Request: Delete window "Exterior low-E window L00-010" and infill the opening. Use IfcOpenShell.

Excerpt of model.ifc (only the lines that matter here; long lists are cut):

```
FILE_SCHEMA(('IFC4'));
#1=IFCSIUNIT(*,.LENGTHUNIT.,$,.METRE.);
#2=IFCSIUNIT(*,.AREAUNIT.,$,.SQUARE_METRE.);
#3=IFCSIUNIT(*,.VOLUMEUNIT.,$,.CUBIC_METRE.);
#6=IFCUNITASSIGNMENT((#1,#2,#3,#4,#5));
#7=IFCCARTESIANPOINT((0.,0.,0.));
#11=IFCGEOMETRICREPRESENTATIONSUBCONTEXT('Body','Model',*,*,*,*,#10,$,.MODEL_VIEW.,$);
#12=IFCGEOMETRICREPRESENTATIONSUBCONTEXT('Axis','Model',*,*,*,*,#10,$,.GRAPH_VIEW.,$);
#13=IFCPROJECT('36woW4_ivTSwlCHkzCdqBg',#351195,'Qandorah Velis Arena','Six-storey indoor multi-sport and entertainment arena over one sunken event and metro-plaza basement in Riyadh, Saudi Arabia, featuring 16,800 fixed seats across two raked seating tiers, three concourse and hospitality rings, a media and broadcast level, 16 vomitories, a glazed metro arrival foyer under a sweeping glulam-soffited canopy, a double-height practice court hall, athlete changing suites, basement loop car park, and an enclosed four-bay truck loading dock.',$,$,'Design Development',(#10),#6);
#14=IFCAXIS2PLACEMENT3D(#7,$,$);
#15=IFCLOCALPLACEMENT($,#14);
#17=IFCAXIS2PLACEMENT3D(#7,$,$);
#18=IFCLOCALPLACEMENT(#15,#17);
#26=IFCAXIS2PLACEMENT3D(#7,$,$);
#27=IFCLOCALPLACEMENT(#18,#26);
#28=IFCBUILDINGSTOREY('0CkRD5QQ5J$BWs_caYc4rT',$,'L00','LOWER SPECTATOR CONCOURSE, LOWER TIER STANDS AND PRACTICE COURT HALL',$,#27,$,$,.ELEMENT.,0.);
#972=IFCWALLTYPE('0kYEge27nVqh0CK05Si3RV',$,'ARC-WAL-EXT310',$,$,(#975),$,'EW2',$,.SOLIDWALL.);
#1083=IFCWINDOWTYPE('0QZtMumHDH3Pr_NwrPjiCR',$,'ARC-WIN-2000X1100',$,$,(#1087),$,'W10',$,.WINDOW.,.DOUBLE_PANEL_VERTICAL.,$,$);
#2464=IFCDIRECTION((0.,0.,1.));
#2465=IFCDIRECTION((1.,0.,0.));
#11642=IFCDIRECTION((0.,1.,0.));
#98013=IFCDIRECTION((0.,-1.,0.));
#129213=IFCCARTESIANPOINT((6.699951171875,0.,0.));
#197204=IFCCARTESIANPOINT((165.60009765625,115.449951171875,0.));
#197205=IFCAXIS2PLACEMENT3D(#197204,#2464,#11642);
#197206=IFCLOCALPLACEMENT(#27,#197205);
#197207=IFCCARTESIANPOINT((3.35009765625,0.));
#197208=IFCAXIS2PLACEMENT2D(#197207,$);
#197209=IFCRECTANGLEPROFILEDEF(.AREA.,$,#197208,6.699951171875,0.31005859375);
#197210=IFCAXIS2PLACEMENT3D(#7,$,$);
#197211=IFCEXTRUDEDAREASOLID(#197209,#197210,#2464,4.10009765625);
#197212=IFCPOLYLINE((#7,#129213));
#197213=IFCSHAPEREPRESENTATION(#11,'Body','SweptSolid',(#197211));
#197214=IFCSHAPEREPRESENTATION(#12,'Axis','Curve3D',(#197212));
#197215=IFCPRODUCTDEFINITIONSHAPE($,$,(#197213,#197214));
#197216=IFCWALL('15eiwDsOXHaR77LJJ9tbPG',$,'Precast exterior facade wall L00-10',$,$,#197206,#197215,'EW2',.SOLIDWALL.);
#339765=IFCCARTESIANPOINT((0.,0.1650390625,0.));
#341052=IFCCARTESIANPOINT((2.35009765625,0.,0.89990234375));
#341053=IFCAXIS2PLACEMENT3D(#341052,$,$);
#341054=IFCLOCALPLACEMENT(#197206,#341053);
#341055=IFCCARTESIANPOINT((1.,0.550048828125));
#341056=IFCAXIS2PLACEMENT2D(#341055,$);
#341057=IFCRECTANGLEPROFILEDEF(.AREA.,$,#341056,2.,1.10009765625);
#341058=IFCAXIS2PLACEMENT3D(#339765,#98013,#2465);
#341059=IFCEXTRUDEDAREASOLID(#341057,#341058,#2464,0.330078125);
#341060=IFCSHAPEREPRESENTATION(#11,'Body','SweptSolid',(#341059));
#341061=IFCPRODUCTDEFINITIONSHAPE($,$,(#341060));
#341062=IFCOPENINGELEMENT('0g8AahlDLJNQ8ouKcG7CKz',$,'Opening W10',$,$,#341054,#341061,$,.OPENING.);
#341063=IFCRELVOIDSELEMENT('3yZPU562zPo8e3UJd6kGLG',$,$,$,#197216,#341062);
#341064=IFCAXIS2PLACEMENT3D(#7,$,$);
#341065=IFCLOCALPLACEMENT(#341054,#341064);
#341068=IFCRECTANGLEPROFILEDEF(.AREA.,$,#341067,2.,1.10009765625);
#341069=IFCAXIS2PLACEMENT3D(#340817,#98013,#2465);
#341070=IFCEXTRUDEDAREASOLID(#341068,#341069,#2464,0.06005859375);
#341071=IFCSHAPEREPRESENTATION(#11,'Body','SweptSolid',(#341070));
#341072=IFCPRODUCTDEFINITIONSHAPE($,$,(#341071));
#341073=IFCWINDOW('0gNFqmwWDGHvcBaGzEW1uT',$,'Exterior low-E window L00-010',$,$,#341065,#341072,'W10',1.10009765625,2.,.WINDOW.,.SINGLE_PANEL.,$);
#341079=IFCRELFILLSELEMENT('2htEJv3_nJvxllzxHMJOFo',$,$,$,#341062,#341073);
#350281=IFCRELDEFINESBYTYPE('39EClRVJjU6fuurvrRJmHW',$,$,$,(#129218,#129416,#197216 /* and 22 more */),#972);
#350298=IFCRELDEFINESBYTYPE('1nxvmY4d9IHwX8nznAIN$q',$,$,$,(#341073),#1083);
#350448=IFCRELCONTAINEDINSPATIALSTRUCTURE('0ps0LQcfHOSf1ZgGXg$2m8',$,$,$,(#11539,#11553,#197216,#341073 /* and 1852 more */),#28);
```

```python
import ifcopenshell
import ifcopenshell.api.feature
import ifcopenshell.api.root
import ifcopenshell.geom
import ifcopenshell.util.shape

model = ifcopenshell.open("model.ifc")
settings = ifcopenshell.geom.settings()


def volume(element):
    """Net volume in cubic metres, openings subtracted."""
    shape = ifcopenshell.geom.create_shape(settings, element)
    return ifcopenshell.util.shape.get_volume(shape.geometry)


window = model.by_id(341073)
opening = window.FillsVoids[0].RelatingOpeningElement
wall = opening.VoidsElements[0].RelatingBuildingElement
before = volume(wall)

ifcopenshell.api.root.remove_product(model, product=window)
ifcopenshell.api.feature.remove_feature(model, feature=opening)

after = volume(wall)

print(f"wall volume {before:.3f} -> {after:.3f} m3")

model.write("model_edited.ifc")
```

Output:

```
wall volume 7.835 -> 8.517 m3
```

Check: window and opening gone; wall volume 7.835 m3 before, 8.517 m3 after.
